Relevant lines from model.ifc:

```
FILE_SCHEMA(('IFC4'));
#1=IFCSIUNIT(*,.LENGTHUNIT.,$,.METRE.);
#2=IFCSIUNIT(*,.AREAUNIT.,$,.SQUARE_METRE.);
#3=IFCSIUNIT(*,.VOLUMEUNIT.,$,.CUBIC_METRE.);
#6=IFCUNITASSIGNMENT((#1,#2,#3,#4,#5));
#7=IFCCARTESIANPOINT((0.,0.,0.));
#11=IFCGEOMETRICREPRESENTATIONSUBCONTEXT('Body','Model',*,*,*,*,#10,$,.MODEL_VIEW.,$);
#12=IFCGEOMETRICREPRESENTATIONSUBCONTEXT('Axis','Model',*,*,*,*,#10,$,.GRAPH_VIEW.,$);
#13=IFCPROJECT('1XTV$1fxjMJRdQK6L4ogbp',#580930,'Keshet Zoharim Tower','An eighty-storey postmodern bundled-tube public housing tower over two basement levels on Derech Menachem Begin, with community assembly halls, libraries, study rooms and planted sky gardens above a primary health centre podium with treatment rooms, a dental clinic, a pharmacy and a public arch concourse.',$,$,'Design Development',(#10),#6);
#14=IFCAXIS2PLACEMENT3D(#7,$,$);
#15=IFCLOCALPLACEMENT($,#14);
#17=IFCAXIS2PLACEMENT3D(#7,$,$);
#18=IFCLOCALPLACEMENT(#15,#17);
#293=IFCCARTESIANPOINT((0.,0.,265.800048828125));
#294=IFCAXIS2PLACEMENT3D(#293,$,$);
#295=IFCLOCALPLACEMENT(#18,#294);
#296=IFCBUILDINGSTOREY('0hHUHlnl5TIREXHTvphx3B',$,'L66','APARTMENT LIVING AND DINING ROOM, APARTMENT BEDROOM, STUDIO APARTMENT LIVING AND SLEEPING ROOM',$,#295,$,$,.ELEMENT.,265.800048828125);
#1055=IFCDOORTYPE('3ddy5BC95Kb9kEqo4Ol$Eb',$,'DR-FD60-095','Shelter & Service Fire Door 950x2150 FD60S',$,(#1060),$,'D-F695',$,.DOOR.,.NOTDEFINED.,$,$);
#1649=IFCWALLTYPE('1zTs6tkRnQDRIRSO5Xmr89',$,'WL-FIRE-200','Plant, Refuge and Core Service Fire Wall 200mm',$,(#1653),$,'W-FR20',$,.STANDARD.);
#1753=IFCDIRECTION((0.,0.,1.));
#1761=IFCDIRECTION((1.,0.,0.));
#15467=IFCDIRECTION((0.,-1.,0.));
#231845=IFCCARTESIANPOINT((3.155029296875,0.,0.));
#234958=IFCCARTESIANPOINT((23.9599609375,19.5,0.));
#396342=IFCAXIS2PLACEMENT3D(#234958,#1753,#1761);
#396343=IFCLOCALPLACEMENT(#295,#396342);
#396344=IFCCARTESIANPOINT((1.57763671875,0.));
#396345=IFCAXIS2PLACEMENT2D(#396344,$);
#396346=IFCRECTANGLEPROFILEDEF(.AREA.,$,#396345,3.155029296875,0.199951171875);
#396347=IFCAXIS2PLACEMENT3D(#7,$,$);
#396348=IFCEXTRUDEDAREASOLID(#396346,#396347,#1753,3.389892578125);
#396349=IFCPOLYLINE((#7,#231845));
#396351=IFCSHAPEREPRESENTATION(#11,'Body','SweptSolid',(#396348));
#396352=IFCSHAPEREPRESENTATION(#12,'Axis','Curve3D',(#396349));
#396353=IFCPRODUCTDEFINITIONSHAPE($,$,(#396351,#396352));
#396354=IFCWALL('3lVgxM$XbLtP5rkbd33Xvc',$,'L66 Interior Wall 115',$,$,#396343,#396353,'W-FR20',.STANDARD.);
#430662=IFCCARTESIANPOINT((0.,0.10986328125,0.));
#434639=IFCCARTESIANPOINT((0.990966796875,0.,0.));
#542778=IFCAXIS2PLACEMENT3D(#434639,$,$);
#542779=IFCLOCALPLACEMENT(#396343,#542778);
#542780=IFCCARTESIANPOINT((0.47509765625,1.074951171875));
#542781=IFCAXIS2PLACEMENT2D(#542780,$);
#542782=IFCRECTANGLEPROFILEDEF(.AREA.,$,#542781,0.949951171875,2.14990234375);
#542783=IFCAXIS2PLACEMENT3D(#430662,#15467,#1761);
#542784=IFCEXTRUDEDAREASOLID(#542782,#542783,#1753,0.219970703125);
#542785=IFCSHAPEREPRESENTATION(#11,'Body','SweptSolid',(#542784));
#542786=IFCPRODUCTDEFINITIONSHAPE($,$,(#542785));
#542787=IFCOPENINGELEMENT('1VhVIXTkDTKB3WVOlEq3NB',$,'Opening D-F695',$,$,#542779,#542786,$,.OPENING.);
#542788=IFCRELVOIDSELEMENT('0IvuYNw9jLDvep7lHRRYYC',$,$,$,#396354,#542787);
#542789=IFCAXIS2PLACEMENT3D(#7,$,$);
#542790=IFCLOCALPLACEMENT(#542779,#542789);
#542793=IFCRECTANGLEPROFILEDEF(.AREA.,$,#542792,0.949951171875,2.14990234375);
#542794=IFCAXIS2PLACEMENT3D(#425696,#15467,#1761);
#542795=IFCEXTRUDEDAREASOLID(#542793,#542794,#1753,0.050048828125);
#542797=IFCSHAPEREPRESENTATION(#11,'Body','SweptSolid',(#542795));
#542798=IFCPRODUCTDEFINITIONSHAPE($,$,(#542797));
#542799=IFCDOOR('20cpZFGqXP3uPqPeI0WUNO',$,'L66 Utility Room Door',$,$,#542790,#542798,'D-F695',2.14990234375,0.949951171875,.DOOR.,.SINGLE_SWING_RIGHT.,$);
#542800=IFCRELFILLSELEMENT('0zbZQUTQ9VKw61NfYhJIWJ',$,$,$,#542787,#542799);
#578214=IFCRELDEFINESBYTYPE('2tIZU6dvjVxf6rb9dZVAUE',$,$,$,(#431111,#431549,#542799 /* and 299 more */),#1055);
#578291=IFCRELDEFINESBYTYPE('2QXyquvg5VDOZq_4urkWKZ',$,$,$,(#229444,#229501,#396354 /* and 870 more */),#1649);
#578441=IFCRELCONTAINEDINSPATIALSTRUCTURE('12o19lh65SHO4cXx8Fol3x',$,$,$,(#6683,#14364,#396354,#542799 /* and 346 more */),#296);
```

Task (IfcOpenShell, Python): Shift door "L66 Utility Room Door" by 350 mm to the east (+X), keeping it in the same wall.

```python
import ifcopenshell
import ifcopenshell.api.geometry
import ifcopenshell.util.placement

model = ifcopenshell.open("model.ifc")

door = model.by_guid("20cpZFGqXP3uPqPeI0WUNO")
opening = door.FillsVoids[0].RelatingOpeningElement
wall = opening.VoidsElements[0].RelatingBuildingElement

wall_matrix = ifcopenshell.util.placement.get_local_placement(wall.ObjectPlacement)
shift = wall_matrix[:3, 0] * 0.35
before = ifcopenshell.util.placement.get_local_placement(door.ObjectPlacement)[:3, 3].copy()

# The door is placed relative to its opening, so it follows when the opening moves.
matrix = ifcopenshell.util.placement.get_local_placement(opening.ObjectPlacement)
matrix[:3, 3] += shift
ifcopenshell.api.geometry.edit_object_placement(
    model, product=opening, matrix=matrix, is_si=False, should_transform_children=True
)

after = ifcopenshell.util.placement.get_local_placement(door.ObjectPlacement)[:3, 3]
print("door moved by", (after - before).round(3) + 0.0)

model.write("model_v2.ifc")
```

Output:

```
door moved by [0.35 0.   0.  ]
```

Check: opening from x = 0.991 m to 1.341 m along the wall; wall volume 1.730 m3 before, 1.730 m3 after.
